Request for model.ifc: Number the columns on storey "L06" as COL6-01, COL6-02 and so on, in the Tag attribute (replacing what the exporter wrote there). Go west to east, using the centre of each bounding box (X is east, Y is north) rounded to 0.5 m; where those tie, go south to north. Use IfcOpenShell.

First a look at what the model holds.

```python
import ifcopenshell
import ifcopenshell.util.element
import ifcopenshell.util.placement

model = ifcopenshell.open("model.ifc")
print(model.schema)
storey = next(s for s in model.by_type("IfcBuildingStorey") if s.Name == "L06")
columns = [e for e in ifcopenshell.util.element.get_decomposition(storey) if e.is_a("IfcColumn")]
for e in sorted(columns, key=lambda e: e.id()):
    origin = ifcopenshell.util.placement.get_local_placement(e.ObjectPlacement)[:3, 3]
    print(e.id(), e.Tag, e.Name, origin.round(2) + 0.0, sep=" | ")
```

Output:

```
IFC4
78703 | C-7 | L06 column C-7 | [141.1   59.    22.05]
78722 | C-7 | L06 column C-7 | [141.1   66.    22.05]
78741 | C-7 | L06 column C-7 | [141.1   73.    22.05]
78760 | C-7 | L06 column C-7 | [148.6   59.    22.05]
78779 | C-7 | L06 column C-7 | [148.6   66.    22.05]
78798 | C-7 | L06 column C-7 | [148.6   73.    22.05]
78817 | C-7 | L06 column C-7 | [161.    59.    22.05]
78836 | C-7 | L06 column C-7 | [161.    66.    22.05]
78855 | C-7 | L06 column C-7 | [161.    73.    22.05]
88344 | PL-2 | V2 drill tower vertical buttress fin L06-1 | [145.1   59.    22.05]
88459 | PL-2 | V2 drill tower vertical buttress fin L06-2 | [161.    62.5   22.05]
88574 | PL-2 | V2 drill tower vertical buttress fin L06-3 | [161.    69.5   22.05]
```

```python
import ifcopenshell
import ifcopenshell.geom
import ifcopenshell.util.element
import ifcopenshell.util.shape

model = ifcopenshell.open("model.ifc")
settings = ifcopenshell.geom.settings()
settings.set("use-world-coords", True)


def centre(element):
    shape = ifcopenshell.geom.create_shape(settings, element)
    return ifcopenshell.util.shape.get_bbox_centroid(shape.geometry)


storey = next(s for s in model.by_type("IfcBuildingStorey") if s.Name == "L06")
columns = [e for e in ifcopenshell.util.element.get_decomposition(storey) if e.is_a("IfcColumn")]

# Insertion points can sit at a corner or the storey origin, so sort by the geometry (in metres).
centres = {e: centre(e) for e in columns}
columns.sort(key=lambda e: (round(centres[e][0] / 0.5), centres[e][1]))

for i, e in enumerate(columns, start=1):
    number = f"COL6-{i:02d}"
    e.Tag = number
    print(e.id(), number)

model.write("model_updated.ifc")
```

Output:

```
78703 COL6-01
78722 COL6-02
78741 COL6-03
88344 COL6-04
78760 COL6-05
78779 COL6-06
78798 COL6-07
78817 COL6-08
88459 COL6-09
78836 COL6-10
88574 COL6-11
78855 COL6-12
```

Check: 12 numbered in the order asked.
